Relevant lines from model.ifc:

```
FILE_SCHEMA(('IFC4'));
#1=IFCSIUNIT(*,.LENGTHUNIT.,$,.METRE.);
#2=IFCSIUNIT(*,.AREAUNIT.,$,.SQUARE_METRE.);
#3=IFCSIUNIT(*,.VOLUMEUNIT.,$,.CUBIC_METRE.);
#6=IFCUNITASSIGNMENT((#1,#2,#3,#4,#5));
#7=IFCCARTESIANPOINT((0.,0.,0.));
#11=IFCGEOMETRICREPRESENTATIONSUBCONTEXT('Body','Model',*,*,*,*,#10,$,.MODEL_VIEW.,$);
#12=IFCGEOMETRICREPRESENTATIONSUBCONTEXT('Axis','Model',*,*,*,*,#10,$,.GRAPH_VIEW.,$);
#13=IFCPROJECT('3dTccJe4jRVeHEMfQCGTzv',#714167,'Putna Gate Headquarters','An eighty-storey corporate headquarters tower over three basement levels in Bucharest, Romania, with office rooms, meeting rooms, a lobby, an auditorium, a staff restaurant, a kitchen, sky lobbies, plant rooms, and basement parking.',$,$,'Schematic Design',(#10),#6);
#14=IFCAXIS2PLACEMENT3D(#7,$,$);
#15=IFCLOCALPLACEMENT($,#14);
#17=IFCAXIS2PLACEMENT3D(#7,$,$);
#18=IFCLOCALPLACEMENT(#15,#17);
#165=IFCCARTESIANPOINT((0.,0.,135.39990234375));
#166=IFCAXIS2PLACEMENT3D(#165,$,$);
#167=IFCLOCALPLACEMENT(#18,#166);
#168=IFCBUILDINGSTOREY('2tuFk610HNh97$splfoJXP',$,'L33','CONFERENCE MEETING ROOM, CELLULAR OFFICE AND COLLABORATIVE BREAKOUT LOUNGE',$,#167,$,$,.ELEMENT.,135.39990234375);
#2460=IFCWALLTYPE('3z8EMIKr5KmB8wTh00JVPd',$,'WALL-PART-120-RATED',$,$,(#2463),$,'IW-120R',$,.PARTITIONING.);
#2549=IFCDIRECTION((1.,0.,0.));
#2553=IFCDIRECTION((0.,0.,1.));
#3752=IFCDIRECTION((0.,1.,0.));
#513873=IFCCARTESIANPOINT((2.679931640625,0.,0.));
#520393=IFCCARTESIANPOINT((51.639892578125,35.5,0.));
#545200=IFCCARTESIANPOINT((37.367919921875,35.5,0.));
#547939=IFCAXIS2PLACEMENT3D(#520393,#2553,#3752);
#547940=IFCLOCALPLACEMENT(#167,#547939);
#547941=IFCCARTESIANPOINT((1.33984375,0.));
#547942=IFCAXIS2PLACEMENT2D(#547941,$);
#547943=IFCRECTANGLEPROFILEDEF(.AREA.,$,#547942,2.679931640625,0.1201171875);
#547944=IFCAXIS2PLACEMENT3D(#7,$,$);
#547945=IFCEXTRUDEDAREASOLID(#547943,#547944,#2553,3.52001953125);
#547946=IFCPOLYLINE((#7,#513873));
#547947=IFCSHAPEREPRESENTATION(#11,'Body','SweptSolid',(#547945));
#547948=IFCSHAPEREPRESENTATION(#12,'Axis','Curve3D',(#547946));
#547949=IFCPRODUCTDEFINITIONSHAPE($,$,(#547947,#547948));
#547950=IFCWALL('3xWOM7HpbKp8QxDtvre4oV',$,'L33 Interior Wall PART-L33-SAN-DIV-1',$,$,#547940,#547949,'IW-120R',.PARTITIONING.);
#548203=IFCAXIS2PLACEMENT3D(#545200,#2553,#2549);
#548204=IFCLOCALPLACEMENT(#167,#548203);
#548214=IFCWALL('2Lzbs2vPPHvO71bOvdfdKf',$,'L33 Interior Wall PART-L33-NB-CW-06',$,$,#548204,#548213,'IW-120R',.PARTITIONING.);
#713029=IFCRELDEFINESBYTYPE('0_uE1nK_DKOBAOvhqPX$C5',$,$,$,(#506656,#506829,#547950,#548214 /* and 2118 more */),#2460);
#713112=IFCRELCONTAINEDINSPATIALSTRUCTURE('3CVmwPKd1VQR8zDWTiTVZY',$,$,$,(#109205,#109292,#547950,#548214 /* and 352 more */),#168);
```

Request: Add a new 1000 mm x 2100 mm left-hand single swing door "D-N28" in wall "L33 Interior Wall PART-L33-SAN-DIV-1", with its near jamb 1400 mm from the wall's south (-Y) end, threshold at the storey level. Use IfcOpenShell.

```python
import numpy as np
import ifcopenshell
import ifcopenshell.api.feature
import ifcopenshell.api.geometry
import ifcopenshell.api.root
import ifcopenshell.api.spatial
import ifcopenshell.geom
import ifcopenshell.util.element
import ifcopenshell.util.placement
import ifcopenshell.util.representation
import ifcopenshell.util.shape
import ifcopenshell.util.unit

model = ifcopenshell.open("model.ifc")
unit_scale = ifcopenshell.util.unit.calculate_unit_scale(model)
settings = ifcopenshell.geom.settings()


def volume(element):
    """Net volume in cubic metres, openings subtracted."""
    shape = ifcopenshell.geom.create_shape(settings, element)
    return ifcopenshell.util.shape.get_volume(shape.geometry)


wall = model.by_guid("3xWOM7HpbKp8QxDtvre4oV")
storey = ifcopenshell.util.element.get_container(wall, ifc_class="IfcBuildingStorey")
context = ifcopenshell.util.representation.get_context(model, "Model", "Body", "MODEL_VIEW")
before = volume(wall)

width, height, from_end, sill = 1, 2.1, 1.4, 0.0  # metres

# The wall runs along its own X axis, and the end named is its -X end.
wall_shape = ifcopenshell.geom.create_shape(settings, wall)
x, y, z = ifcopenshell.util.shape.get_vertices(wall_shape.geometry).T
start = x.min() + from_end
face, thickness = float(y.min()), float(y.max() - y.min())
wall_matrix = ifcopenshell.util.placement.get_local_placement(wall.ObjectPlacement)
level = ifcopenshell.util.placement.get_local_placement(storey.ObjectPlacement)[2, 3]


def in_wall(x, y):
    """Placement at x, y metres in the wall's axes, at sill height."""
    matrix = wall_matrix.copy()
    matrix[:, 3] = wall_matrix @ np.array([x / unit_scale, y / unit_scale, 0.0, 1.0])
    matrix[2, 3] = level + sill / unit_scale
    return matrix


# Opening: a box that overshoots both wall faces by 50 mm.
opening = ifcopenshell.api.root.create_entity(model, ifc_class="IfcOpeningElement", predefined_type="OPENING")
box = ifcopenshell.api.geometry.add_wall_representation(
    model, context=context, length=width, height=height, thickness=thickness + 0.1
)
ifcopenshell.api.geometry.assign_representation(model, product=opening, representation=box)
ifcopenshell.api.geometry.edit_object_placement(model, product=opening, matrix=in_wall(start, face - 0.05), is_si=False)
ifcopenshell.api.feature.add_feature(model, feature=opening, element=wall)

door = ifcopenshell.api.root.create_entity(model, ifc_class="IfcDoor", name="D-N28", predefined_type="DOOR")
door.OverallWidth, door.OverallHeight = width / unit_scale, height / unit_scale
door.OperationType = "SINGLE_SWING_LEFT"
body = ifcopenshell.api.geometry.add_door_representation(
    model,
    context=context,
    overall_width=door.OverallWidth,
    overall_height=door.OverallHeight,
    operation_type="SINGLE_SWING_LEFT",
    lining_properties={"LiningDepth": thickness / unit_scale, "ThresholdDepth": thickness / unit_scale},
)
ifcopenshell.api.geometry.assign_representation(model, product=door, representation=body)
ifcopenshell.api.spatial.assign_container(model, products=[door], relating_structure=storey)
ifcopenshell.api.feature.add_filling(model, opening=opening, element=door)

# The lining spans the wall, so the door starts at the wall face.
ifcopenshell.api.geometry.edit_object_placement(model, product=door, matrix=in_wall(start, face), is_si=False)

after = volume(wall)

print(f"wall volume {before:.3f} -> {after:.3f} m3")

model.write("model_edited.ifc")
```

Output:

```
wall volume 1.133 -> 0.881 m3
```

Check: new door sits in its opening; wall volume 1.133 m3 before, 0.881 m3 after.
